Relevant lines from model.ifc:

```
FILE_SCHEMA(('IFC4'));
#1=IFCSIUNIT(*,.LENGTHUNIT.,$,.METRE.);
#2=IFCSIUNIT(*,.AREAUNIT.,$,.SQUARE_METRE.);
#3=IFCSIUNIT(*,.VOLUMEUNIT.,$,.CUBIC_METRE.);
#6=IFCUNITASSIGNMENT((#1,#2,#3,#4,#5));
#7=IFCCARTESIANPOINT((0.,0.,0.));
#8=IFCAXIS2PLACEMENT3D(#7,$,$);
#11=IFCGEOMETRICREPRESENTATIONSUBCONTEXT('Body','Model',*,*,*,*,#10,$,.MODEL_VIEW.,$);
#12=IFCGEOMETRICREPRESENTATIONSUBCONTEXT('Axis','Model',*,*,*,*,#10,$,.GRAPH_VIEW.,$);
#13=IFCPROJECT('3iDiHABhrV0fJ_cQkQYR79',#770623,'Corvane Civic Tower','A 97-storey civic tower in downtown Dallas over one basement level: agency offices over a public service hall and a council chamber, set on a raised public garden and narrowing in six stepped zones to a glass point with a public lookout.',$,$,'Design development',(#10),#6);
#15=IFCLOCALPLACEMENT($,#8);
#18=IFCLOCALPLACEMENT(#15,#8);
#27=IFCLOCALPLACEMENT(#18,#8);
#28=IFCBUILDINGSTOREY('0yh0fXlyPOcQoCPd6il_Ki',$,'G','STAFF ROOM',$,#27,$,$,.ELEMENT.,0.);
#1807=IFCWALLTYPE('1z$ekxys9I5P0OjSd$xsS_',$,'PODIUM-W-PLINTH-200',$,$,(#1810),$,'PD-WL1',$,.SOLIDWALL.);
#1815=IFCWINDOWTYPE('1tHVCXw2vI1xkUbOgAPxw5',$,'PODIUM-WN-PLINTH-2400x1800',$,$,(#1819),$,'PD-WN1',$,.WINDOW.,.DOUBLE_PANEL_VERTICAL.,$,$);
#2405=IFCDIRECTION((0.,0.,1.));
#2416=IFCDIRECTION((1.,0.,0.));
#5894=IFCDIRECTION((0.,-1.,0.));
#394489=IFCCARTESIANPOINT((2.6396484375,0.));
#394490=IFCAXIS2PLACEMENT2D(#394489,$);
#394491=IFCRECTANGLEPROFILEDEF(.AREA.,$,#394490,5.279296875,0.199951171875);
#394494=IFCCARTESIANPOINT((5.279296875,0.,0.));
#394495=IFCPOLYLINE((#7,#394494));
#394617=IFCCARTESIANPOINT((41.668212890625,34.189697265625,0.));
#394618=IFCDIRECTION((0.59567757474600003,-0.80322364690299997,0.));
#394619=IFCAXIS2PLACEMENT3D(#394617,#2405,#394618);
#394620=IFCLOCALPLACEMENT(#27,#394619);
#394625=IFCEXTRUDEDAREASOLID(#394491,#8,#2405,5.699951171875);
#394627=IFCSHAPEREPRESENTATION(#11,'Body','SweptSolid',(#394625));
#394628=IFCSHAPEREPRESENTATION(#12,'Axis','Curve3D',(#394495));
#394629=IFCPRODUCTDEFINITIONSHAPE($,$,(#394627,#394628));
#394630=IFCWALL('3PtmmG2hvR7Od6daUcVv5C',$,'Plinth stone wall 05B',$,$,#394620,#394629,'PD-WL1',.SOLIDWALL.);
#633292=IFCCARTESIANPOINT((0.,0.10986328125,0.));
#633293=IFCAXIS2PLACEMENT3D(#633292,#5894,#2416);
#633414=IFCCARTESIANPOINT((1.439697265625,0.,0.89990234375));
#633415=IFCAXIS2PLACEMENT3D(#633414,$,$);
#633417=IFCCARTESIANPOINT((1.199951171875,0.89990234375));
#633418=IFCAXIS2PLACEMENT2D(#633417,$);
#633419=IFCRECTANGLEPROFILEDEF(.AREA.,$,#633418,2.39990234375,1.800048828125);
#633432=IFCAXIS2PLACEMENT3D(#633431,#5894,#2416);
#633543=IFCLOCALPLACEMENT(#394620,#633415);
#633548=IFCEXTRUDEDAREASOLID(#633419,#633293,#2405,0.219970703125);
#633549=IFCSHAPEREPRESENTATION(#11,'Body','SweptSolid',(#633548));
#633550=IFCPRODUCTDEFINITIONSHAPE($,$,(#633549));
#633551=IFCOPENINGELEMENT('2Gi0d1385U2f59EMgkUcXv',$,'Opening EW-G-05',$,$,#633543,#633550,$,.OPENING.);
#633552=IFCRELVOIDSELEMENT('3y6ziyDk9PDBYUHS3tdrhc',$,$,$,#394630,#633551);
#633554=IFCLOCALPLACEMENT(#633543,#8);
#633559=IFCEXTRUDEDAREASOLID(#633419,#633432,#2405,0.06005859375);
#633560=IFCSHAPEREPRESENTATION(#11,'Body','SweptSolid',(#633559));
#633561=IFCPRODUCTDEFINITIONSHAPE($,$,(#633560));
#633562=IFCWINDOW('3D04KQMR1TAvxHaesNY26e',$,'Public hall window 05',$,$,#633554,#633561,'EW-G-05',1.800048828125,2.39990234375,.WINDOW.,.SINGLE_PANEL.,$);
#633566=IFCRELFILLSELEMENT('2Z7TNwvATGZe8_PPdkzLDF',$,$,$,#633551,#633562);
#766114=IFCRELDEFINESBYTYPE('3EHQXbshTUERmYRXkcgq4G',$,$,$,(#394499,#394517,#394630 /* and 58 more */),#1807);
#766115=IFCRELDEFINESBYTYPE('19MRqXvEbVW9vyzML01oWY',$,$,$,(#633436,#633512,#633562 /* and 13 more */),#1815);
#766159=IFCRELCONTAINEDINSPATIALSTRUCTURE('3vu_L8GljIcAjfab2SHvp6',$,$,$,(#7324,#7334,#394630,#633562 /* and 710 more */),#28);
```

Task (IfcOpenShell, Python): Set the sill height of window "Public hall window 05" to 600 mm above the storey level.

```python
import numpy as np
import ifcopenshell
import ifcopenshell.api.geometry
import ifcopenshell.geom
import ifcopenshell.util.element
import ifcopenshell.util.placement
import ifcopenshell.util.shape
import ifcopenshell.util.unit

model = ifcopenshell.open("model.ifc")
unit_scale = ifcopenshell.util.unit.calculate_unit_scale(model)

window = model.by_id(633562)
opening = window.FillsVoids[0].RelatingOpeningElement
storey = ifcopenshell.util.element.get_container(window, ifc_class="IfcBuildingStorey")
level = ifcopenshell.util.placement.get_local_placement(storey.ObjectPlacement)[2, 3]

# The opening's origin need not be at the sill, so measure its lowest point.
shape = ifcopenshell.geom.create_shape(ifcopenshell.geom.settings(), opening)
bottom = ifcopenshell.util.shape.get_shape_bottom_elevation(shape, shape.geometry) / unit_scale
dz = level + 0.6 - bottom

shift = np.array([0.0, 0.0, dz])
# The window is placed relative to its opening, so it follows when the opening moves.
matrix = ifcopenshell.util.placement.get_local_placement(opening.ObjectPlacement)
matrix[:3, 3] += shift
ifcopenshell.api.geometry.edit_object_placement(
    model, product=opening, matrix=matrix, is_si=False, should_transform_children=True
)

print(f"moved by {dz * unit_scale:+.3f} m")

model.write("model_rev.ifc")
```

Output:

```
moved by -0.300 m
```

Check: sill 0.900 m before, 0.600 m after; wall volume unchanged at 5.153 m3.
